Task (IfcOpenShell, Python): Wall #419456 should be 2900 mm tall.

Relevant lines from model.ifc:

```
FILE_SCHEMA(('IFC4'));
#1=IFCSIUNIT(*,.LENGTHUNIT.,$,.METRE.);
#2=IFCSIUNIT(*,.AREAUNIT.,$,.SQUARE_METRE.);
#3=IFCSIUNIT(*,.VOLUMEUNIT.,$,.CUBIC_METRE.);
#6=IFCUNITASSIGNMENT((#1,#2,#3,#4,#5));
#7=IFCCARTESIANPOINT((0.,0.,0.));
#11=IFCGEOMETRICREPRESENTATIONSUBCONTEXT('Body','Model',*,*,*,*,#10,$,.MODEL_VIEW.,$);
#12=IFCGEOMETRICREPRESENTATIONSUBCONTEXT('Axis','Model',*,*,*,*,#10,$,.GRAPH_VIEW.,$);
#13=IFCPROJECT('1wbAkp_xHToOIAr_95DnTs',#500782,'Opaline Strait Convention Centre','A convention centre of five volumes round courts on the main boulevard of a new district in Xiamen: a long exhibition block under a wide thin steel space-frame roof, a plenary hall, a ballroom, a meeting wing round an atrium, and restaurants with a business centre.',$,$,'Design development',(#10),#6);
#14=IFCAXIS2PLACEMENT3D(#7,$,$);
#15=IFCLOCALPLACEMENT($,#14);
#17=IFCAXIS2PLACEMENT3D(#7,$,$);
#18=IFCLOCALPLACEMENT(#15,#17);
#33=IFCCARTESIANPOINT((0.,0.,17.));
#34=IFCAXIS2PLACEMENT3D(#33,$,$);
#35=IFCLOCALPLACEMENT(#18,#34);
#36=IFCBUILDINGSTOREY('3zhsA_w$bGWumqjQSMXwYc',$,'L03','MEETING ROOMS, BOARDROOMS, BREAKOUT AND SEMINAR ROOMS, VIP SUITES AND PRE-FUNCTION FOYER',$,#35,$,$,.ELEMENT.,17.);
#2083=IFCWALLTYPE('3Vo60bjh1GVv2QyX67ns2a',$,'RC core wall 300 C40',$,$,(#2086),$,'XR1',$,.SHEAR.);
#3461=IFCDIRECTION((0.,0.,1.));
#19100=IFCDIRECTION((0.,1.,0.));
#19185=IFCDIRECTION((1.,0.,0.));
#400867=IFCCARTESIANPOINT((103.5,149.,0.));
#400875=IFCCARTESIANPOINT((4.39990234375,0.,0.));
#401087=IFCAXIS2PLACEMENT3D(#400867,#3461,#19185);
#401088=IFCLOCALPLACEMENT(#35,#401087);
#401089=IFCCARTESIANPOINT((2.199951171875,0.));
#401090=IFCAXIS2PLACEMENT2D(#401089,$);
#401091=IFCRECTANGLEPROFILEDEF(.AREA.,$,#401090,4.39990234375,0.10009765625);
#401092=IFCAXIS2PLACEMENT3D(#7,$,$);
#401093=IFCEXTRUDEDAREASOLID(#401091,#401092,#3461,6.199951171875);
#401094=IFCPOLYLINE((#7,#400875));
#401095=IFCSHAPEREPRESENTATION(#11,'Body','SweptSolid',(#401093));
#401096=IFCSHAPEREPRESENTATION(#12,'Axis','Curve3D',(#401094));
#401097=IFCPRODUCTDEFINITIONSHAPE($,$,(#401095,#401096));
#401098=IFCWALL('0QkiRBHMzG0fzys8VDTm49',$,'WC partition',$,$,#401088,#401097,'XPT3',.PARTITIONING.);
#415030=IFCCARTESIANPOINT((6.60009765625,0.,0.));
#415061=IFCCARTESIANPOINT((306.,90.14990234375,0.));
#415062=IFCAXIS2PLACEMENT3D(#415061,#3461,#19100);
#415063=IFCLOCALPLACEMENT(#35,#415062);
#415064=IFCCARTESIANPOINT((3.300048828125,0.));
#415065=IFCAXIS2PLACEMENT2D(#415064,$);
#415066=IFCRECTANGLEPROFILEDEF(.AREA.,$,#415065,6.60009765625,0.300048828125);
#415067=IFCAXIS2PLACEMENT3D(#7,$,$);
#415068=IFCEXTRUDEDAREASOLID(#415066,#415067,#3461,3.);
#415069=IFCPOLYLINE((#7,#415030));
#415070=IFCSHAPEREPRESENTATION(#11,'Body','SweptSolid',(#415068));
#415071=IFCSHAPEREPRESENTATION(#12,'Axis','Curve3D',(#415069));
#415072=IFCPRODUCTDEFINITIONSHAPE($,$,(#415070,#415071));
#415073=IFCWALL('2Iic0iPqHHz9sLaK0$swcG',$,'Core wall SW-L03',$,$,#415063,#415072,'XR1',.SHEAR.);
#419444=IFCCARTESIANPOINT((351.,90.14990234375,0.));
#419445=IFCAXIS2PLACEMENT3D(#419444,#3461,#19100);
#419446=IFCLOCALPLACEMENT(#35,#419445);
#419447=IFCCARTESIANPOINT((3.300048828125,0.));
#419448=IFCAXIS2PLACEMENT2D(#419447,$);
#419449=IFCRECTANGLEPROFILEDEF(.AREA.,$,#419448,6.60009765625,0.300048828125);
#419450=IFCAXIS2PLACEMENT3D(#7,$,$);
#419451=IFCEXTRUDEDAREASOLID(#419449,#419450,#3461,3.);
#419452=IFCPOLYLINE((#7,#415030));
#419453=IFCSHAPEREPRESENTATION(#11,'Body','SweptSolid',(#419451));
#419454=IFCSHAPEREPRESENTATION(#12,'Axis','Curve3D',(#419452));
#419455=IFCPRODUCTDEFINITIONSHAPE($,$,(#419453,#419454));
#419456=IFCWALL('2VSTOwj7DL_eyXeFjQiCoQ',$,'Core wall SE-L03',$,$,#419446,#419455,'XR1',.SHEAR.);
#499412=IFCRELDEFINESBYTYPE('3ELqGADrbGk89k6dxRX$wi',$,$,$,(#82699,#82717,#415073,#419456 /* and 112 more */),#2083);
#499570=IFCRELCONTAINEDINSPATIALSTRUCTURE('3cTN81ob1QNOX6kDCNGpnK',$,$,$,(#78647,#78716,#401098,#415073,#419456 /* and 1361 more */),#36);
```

```python
import ifcopenshell
import ifcopenshell.geom
import ifcopenshell.util.representation
import ifcopenshell.util.shape

model = ifcopenshell.open("model.ifc")
settings = ifcopenshell.geom.settings()


def volume(element):
    """Net volume in cubic metres, openings subtracted."""
    shape = ifcopenshell.geom.create_shape(settings, element)
    return ifcopenshell.util.shape.get_volume(shape.geometry)


wall = model.by_id(419456)
before = volume(wall)

body = ifcopenshell.util.representation.get_representation(wall, "Model", "Body")
solid = body.Items[0]
old_height = solid.Depth
solid.Depth = 2.9
after = volume(wall)

print(f"height {old_height:g} -> {solid.Depth:g}, volume {before:.3f} -> {after:.3f} m3")

model.write("model_v2.ifc")
```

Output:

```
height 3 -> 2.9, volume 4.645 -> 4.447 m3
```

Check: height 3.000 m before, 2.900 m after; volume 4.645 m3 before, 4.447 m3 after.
